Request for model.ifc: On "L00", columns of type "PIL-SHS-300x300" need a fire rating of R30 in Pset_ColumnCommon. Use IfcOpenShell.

First a look at what the model holds.

```python
import ifcopenshell
import ifcopenshell.util.element

model = ifcopenshell.open("model.ifc")
print(model.schema)
storey = next(s for s in model.by_type("IfcBuildingStorey") if s.Name == "L00")
columns = [e for e in ifcopenshell.util.element.get_decomposition(storey) if e.is_a("IfcColumn")]
seen = {}
for e in columns:
    element_type = ifcopenshell.util.element.get_type(e)
    key = (element_type.Name if element_type != e and element_type else None, ifcopenshell.util.element.get_pset(e, "Pset_ColumnCommon", "FireRating"))
    seen[key] = seen.get(key, 0) + 1
for (name, value), count in sorted(seen.items(), key=str):
    print(count, "x", name, "|", value)
```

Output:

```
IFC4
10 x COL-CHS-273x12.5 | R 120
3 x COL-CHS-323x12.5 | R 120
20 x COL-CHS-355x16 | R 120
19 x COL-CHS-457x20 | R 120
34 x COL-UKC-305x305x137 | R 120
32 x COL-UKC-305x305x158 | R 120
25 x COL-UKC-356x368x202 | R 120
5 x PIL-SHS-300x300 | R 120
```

```python
import ifcopenshell
import ifcopenshell.api.pset
import ifcopenshell.util.element

model = ifcopenshell.open("model.ifc")

storey = next(s for s in model.by_type("IfcBuildingStorey") if s.Name == "L00")
columns = [e for e in ifcopenshell.util.element.get_decomposition(storey) if e.is_a("IfcColumn")]

count = 0
for e in columns:
    element_type = ifcopenshell.util.element.get_type(e)
    if element_type in (None, e) or element_type.Name != "PIL-SHS-300x300":
        continue
    # add_pset returns the element's existing set when there is one.
    pset = ifcopenshell.api.pset.add_pset(model, product=e, name="Pset_ColumnCommon")
    ifcopenshell.api.pset.edit_pset(model, pset=pset, properties={"FireRating": "R30"})
    count += 1

print(count, "columns updated")

model.write("model_rev.ifc")
```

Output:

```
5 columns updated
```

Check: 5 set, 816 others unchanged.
